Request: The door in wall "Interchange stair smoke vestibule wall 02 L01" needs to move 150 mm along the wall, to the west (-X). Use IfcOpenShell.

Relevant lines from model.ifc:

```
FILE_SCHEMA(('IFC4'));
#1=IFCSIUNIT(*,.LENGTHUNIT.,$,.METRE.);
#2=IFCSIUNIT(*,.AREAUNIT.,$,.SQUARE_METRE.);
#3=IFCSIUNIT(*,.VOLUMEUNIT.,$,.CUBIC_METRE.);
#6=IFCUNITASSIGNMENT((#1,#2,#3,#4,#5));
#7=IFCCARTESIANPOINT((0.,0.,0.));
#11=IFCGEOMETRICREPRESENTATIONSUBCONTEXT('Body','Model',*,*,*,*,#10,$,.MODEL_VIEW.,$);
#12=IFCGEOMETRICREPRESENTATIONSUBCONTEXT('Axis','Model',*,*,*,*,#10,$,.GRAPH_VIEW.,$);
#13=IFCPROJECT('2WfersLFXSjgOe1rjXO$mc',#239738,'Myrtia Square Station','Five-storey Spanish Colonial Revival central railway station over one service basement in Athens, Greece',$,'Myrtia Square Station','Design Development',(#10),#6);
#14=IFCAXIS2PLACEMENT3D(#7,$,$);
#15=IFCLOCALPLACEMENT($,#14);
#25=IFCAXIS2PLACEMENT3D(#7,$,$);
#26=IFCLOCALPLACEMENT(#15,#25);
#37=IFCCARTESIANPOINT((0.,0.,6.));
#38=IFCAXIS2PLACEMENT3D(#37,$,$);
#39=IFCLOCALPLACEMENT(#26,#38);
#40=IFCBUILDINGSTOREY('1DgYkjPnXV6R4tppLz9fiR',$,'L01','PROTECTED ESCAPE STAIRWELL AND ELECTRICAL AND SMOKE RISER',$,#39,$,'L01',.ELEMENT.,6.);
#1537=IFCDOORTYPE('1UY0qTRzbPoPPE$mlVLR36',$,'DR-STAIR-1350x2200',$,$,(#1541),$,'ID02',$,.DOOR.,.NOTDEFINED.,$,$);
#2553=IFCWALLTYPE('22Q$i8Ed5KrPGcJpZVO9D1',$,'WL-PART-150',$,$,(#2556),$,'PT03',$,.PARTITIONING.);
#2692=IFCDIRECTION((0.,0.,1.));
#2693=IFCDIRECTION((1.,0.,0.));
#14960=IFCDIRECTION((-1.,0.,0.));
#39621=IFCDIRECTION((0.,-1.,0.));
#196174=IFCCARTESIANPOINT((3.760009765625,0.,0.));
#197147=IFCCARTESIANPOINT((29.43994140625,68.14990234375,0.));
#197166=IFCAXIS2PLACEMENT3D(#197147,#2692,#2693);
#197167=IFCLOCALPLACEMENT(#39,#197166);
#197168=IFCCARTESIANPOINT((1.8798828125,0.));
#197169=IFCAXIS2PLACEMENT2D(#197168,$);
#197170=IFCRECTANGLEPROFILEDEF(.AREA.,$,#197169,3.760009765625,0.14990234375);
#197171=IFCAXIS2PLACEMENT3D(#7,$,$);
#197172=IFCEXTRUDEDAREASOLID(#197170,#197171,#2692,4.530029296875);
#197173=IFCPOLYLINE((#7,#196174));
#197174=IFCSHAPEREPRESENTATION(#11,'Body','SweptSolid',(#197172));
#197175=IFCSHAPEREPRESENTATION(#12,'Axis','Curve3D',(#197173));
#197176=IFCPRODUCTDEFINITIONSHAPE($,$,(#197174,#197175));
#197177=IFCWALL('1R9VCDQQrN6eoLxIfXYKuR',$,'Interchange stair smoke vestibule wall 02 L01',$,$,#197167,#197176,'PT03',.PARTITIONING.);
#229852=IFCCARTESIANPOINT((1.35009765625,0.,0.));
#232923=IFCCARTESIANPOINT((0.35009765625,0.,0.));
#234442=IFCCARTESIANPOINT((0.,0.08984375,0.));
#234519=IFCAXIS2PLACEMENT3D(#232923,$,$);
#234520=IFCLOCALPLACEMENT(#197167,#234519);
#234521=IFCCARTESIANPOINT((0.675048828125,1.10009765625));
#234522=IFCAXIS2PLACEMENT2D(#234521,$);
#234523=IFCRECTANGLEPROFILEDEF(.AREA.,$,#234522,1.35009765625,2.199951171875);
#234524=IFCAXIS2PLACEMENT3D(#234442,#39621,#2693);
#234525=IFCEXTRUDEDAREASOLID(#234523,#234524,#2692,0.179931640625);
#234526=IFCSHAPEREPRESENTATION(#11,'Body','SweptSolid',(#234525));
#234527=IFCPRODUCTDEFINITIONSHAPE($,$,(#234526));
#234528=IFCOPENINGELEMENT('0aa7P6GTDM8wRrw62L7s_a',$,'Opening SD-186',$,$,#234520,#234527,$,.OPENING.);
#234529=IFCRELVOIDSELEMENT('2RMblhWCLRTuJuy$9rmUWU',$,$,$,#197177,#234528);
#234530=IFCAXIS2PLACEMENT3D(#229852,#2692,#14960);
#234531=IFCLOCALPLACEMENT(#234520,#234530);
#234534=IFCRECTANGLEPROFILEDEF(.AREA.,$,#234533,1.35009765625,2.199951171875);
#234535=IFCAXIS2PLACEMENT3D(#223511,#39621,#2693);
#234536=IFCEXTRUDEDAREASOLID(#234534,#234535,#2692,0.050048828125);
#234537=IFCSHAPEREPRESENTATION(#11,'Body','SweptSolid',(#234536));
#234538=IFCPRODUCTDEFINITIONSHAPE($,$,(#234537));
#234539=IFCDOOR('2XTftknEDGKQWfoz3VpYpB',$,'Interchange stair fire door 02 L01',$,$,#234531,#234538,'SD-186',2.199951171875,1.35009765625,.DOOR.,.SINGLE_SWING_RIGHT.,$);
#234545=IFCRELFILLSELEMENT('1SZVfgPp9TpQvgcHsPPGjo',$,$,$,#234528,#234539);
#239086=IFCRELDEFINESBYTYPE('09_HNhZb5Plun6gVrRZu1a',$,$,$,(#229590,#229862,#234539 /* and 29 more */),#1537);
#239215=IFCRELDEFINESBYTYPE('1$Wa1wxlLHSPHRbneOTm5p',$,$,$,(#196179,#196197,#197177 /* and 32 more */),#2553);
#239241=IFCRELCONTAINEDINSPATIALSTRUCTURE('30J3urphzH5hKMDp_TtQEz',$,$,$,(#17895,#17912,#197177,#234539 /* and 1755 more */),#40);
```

```python
import ifcopenshell
import ifcopenshell.api.geometry
import ifcopenshell.util.placement
import ifcopenshell.util.unit

model = ifcopenshell.open("model.ifc")
unit_scale = ifcopenshell.util.unit.calculate_unit_scale(model)

door = model.by_guid("2XTftknEDGKQWfoz3VpYpB")
opening = door.FillsVoids[0].RelatingOpeningElement
wall = opening.VoidsElements[0].RelatingBuildingElement

wall_matrix = ifcopenshell.util.placement.get_local_placement(wall.ObjectPlacement)
shift = wall_matrix[:3, 0] * -0.15 / unit_scale
before = ifcopenshell.util.placement.get_local_placement(door.ObjectPlacement)[:3, 3].copy()

# The door is placed relative to its opening, so it follows when the opening moves.
matrix = ifcopenshell.util.placement.get_local_placement(opening.ObjectPlacement)
matrix[:3, 3] += shift
ifcopenshell.api.geometry.edit_object_placement(
    model, product=opening, matrix=matrix, is_si=False, should_transform_children=True
)

after = ifcopenshell.util.placement.get_local_placement(door.ObjectPlacement)[:3, 3]
print("door moved by", (after - before).round(3) + 0.0)

model.write("model-out.ifc")
```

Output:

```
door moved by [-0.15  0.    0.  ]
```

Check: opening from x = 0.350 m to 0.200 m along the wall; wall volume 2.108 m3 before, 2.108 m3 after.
